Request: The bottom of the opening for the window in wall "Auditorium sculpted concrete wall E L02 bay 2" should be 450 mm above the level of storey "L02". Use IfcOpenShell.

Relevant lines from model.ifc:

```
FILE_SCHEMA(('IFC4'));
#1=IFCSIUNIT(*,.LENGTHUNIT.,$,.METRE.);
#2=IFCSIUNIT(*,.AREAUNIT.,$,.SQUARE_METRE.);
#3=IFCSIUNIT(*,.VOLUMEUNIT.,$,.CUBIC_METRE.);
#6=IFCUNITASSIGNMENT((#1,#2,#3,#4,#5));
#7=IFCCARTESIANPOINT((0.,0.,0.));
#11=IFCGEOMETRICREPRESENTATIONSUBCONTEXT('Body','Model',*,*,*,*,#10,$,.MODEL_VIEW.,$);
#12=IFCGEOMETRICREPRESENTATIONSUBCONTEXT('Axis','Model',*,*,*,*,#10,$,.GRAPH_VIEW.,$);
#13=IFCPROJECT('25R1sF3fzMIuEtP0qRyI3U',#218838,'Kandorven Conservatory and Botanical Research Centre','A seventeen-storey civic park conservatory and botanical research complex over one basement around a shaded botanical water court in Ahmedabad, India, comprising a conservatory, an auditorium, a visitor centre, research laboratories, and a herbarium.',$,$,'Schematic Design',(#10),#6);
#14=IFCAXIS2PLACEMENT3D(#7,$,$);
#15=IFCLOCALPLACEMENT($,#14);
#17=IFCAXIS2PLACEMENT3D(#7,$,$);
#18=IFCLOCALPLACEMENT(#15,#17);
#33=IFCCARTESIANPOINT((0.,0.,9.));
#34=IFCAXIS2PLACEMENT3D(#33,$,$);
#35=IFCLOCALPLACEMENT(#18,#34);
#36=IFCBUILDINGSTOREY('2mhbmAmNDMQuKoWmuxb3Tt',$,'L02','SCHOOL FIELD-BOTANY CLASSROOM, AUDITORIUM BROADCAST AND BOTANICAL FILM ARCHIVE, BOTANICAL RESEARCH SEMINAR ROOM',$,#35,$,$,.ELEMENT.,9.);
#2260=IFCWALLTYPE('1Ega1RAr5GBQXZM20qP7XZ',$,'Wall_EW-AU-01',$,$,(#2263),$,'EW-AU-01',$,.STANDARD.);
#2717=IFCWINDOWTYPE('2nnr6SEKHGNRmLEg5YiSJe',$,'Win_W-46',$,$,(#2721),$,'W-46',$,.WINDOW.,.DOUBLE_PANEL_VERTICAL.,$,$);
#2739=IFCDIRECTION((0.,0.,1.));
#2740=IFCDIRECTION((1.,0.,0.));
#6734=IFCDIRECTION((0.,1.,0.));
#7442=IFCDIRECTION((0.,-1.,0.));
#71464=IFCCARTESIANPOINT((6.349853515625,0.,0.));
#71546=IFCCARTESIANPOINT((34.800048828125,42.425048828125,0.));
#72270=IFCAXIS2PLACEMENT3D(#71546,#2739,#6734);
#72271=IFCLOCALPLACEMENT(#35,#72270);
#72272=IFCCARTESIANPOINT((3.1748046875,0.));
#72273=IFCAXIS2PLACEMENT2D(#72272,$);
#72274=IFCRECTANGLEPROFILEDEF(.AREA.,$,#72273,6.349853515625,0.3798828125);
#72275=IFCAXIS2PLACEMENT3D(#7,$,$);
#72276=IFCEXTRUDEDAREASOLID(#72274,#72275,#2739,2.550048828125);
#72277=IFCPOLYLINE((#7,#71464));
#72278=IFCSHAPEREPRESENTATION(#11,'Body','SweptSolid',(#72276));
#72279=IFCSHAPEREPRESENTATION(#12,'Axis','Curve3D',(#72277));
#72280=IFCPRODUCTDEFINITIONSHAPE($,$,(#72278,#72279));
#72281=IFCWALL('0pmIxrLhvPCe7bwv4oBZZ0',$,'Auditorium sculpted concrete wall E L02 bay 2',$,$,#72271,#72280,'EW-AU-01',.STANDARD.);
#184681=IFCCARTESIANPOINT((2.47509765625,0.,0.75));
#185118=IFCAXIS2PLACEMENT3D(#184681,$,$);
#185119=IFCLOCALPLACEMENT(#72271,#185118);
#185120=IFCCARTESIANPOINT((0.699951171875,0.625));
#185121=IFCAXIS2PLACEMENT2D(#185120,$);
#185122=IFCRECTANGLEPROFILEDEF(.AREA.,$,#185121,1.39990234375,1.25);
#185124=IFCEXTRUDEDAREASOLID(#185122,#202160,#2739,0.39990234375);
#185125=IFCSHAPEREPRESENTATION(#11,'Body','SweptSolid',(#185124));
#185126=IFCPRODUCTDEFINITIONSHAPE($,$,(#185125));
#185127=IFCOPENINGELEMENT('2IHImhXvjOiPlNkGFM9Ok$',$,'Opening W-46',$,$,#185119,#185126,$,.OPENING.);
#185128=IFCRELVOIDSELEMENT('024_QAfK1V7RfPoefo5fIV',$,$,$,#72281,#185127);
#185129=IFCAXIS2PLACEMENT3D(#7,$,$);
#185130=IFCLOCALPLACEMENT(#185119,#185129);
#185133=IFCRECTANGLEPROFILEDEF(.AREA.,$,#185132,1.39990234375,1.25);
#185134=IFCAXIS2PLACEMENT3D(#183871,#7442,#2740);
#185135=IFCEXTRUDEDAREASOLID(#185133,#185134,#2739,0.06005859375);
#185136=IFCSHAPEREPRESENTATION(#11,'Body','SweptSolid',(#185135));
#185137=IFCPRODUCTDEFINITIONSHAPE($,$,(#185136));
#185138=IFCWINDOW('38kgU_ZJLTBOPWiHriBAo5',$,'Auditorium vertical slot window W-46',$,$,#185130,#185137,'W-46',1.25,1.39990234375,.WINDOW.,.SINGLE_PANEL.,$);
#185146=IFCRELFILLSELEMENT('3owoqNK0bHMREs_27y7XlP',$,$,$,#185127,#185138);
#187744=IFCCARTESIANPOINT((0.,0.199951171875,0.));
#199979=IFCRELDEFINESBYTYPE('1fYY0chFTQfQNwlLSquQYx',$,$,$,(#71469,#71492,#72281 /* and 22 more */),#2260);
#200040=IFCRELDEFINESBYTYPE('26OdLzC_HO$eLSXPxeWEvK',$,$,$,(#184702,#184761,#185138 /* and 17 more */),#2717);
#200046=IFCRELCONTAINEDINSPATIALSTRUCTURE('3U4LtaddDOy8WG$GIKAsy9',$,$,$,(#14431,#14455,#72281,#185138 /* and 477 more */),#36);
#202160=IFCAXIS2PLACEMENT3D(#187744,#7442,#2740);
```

```python
import numpy as np
import ifcopenshell
import ifcopenshell.api.geometry
import ifcopenshell.geom
import ifcopenshell.util.element
import ifcopenshell.util.placement
import ifcopenshell.util.shape
import ifcopenshell.util.unit

model = ifcopenshell.open("model.ifc")
unit_scale = ifcopenshell.util.unit.calculate_unit_scale(model)

window = model.by_id(185138)
opening = window.FillsVoids[0].RelatingOpeningElement
storey = ifcopenshell.util.element.get_container(window, ifc_class="IfcBuildingStorey")
level = ifcopenshell.util.placement.get_local_placement(storey.ObjectPlacement)[2, 3]

# The opening's origin need not be at the sill, so measure its lowest point.
shape = ifcopenshell.geom.create_shape(ifcopenshell.geom.settings(), opening)
bottom = ifcopenshell.util.shape.get_shape_bottom_elevation(shape, shape.geometry) / unit_scale
dz = level + 0.45 / unit_scale - bottom

shift = np.array([0.0, 0.0, dz])
# The window is placed relative to its opening, so it follows when the opening moves.
matrix = ifcopenshell.util.placement.get_local_placement(opening.ObjectPlacement)
matrix[:3, 3] += shift
ifcopenshell.api.geometry.edit_object_placement(
    model, product=opening, matrix=matrix, is_si=False, should_transform_children=True
)

print(f"moved by {dz * unit_scale:+.3f} m")

model.write("model-out.ifc")
```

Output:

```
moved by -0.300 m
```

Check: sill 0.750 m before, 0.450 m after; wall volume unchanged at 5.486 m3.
